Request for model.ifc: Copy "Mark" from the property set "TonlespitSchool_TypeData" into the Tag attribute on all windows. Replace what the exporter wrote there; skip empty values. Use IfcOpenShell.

First a look at what the model holds.

```python
import ifcopenshell
import ifcopenshell.util.element

model = ifcopenshell.open("model.ifc")
print(model.schema)
windows = model.by_type("IfcWindow")
print(len(windows), "windows")
for e in windows[:8]:
    source = ifcopenshell.util.element.get_pset(e, "TonlespitSchool_TypeData", "Mark")
    target = e.Tag
    print(e.id(), repr(source), repr(target), sep=" | ")
```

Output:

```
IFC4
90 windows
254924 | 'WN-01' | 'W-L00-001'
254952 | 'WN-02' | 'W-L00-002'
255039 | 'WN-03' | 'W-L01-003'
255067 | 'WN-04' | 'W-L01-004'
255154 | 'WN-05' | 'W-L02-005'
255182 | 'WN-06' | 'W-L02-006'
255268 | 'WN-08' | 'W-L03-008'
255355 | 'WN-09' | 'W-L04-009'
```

```python
import ifcopenshell
import ifcopenshell.util.element

model = ifcopenshell.open("model.ifc")

count = 0
for e in model.by_type("IfcWindow"):
    value = ifcopenshell.util.element.get_pset(e, "TonlespitSchool_TypeData", "Mark")
    current = e.Tag
    if not value or not value.strip() or current == value:
        continue
    e.Tag = value
    count += 1

print(count, "windows updated")

model.write("model_updated.ifc")
```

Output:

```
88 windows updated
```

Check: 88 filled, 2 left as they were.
